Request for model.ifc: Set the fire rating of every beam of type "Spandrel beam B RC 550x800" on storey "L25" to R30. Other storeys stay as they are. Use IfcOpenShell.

First a look at what the model holds.

```python
import ifcopenshell
import ifcopenshell.util.element

model = ifcopenshell.open("model.ifc")
print(model.schema)
storey = next(s for s in model.by_type("IfcBuildingStorey") if s.Name == "L25")
beams = [e for e in ifcopenshell.util.element.get_decomposition(storey) if e.is_a("IfcBeam")]
seen = {}
for e in beams:
    element_type = ifcopenshell.util.element.get_type(e)
    key = (element_type.Name if element_type != e and element_type else None, ifcopenshell.util.element.get_pset(e, "Pset_BeamCommon", "FireRating"))
    seen[key] = seen.get(key, 0) + 1
for (name, value), count in sorted(seen.items(), key=str):
    print(count, "x", name, "|", value)
```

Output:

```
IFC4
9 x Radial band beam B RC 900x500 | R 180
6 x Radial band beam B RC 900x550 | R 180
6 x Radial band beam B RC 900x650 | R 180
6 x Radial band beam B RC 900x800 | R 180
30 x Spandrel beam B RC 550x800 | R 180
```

```python
import ifcopenshell
import ifcopenshell.api.pset
import ifcopenshell.util.element

model = ifcopenshell.open("model.ifc")

storey = next(s for s in model.by_type("IfcBuildingStorey") if s.Name == "L25")
beams = [e for e in ifcopenshell.util.element.get_decomposition(storey) if e.is_a("IfcBeam")]

count = 0
for e in beams:
    element_type = ifcopenshell.util.element.get_type(e)
    if element_type in (None, e) or element_type.Name != "Spandrel beam B RC 550x800":
        continue
    found = ifcopenshell.util.element.get_pset(e, "Pset_BeamCommon", should_inherit=False)
    if found:
        pset = model.by_id(found["id"])
        if len(ifcopenshell.util.element.get_elements_by_pset(pset)) > 1:
            pset = ifcopenshell.api.pset.unshare_pset(model, products=[e], pset=pset)[0]
    else:
        pset = ifcopenshell.api.pset.add_pset(model, product=e, name="Pset_BeamCommon")
    ifcopenshell.api.pset.edit_pset(model, pset=pset, properties={"FireRating": "R30"})
    count += 1

print(count, "beams updated")

model.write("model-out.ifc")
```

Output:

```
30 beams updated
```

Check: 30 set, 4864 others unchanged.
